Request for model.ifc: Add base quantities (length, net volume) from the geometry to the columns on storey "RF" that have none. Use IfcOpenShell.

First a look at what the model holds.

```python
import ifcopenshell
import ifcopenshell.util.element
import ifcopenshell.util.unit

model = ifcopenshell.open("model.ifc")
print(model.schema)
for unit_type in ("LENGTHUNIT", "AREAUNIT", "VOLUMEUNIT"):
    print(unit_type, ifcopenshell.util.unit.calculate_unit_scale(model, unit_type))
storey = next(s for s in model.by_type("IfcBuildingStorey") if s.Name == "RF")
columns = [e for e in ifcopenshell.util.element.get_decomposition(storey) if e.is_a("IfcColumn")]
for e in sorted(columns, key=lambda e: e.id()):
    print(e.id(), e.is_a(), e.Name, list(ifcopenshell.util.element.get_psets(e, qtos_only=True)), sep=" | ")
```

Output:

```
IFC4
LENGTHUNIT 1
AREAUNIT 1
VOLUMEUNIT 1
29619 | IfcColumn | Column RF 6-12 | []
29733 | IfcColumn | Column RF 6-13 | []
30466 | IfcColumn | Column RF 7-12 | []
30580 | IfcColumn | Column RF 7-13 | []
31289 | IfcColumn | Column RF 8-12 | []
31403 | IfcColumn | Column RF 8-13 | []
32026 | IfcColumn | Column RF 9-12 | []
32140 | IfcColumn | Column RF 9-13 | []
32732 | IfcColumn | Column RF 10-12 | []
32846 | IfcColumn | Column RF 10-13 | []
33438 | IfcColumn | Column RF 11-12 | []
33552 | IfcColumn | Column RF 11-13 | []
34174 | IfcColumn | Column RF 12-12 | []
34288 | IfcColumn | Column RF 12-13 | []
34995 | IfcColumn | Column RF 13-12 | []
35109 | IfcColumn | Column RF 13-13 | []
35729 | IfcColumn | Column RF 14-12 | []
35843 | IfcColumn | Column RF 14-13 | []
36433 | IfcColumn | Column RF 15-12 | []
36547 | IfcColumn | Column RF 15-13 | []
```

```python
import ifcopenshell
import ifcopenshell.api.pset
import ifcopenshell.geom
import ifcopenshell.util.element
import ifcopenshell.util.shape
import ifcopenshell.util.unit

model = ifcopenshell.open("model.ifc")
unit_scale = ifcopenshell.util.unit.calculate_unit_scale(model)
volume_scale = ifcopenshell.util.unit.calculate_unit_scale(model, "VOLUMEUNIT")
settings = ifcopenshell.geom.settings()

storey = next(s for s in model.by_type("IfcBuildingStorey") if s.Name == "RF")
columns = [e for e in ifcopenshell.util.element.get_decomposition(storey) if e.is_a("IfcColumn")]

for e in sorted(columns, key=lambda e: e.id()):
    if ifcopenshell.util.element.get_psets(e, qtos_only=True, should_inherit=False):
        continue
    # Geometry comes back in metres, in the element's own axes.
    shape = ifcopenshell.geom.create_shape(settings, e)
    values = {
        "Length": ifcopenshell.util.shape.get_z(shape.geometry) / unit_scale,
        "NetVolume": ifcopenshell.util.shape.get_volume(shape.geometry) / volume_scale,
    }
    qto = ifcopenshell.api.pset.add_qto(model, product=e, name="Qto_ColumnBaseQuantities")
    ifcopenshell.api.pset.edit_qto(model, qto=qto, properties=values)
    print(e.id(), {k: round(v, 3) for k, v in values.items()})

model.write("model_edited.ifc")
```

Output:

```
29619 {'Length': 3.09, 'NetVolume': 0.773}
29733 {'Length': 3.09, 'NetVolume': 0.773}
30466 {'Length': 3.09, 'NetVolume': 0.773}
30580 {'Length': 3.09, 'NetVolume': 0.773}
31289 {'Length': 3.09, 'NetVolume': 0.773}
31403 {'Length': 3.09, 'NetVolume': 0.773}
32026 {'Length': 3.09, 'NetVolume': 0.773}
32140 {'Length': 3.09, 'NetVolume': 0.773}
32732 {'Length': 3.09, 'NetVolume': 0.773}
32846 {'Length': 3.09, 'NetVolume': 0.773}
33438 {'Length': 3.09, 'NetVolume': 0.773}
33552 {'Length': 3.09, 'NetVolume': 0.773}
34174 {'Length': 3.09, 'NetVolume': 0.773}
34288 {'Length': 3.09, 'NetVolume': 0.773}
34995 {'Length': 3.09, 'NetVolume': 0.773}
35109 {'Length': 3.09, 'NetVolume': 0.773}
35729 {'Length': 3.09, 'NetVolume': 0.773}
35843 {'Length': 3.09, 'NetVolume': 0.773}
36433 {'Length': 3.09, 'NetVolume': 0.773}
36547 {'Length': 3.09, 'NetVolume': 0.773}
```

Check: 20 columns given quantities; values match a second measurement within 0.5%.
